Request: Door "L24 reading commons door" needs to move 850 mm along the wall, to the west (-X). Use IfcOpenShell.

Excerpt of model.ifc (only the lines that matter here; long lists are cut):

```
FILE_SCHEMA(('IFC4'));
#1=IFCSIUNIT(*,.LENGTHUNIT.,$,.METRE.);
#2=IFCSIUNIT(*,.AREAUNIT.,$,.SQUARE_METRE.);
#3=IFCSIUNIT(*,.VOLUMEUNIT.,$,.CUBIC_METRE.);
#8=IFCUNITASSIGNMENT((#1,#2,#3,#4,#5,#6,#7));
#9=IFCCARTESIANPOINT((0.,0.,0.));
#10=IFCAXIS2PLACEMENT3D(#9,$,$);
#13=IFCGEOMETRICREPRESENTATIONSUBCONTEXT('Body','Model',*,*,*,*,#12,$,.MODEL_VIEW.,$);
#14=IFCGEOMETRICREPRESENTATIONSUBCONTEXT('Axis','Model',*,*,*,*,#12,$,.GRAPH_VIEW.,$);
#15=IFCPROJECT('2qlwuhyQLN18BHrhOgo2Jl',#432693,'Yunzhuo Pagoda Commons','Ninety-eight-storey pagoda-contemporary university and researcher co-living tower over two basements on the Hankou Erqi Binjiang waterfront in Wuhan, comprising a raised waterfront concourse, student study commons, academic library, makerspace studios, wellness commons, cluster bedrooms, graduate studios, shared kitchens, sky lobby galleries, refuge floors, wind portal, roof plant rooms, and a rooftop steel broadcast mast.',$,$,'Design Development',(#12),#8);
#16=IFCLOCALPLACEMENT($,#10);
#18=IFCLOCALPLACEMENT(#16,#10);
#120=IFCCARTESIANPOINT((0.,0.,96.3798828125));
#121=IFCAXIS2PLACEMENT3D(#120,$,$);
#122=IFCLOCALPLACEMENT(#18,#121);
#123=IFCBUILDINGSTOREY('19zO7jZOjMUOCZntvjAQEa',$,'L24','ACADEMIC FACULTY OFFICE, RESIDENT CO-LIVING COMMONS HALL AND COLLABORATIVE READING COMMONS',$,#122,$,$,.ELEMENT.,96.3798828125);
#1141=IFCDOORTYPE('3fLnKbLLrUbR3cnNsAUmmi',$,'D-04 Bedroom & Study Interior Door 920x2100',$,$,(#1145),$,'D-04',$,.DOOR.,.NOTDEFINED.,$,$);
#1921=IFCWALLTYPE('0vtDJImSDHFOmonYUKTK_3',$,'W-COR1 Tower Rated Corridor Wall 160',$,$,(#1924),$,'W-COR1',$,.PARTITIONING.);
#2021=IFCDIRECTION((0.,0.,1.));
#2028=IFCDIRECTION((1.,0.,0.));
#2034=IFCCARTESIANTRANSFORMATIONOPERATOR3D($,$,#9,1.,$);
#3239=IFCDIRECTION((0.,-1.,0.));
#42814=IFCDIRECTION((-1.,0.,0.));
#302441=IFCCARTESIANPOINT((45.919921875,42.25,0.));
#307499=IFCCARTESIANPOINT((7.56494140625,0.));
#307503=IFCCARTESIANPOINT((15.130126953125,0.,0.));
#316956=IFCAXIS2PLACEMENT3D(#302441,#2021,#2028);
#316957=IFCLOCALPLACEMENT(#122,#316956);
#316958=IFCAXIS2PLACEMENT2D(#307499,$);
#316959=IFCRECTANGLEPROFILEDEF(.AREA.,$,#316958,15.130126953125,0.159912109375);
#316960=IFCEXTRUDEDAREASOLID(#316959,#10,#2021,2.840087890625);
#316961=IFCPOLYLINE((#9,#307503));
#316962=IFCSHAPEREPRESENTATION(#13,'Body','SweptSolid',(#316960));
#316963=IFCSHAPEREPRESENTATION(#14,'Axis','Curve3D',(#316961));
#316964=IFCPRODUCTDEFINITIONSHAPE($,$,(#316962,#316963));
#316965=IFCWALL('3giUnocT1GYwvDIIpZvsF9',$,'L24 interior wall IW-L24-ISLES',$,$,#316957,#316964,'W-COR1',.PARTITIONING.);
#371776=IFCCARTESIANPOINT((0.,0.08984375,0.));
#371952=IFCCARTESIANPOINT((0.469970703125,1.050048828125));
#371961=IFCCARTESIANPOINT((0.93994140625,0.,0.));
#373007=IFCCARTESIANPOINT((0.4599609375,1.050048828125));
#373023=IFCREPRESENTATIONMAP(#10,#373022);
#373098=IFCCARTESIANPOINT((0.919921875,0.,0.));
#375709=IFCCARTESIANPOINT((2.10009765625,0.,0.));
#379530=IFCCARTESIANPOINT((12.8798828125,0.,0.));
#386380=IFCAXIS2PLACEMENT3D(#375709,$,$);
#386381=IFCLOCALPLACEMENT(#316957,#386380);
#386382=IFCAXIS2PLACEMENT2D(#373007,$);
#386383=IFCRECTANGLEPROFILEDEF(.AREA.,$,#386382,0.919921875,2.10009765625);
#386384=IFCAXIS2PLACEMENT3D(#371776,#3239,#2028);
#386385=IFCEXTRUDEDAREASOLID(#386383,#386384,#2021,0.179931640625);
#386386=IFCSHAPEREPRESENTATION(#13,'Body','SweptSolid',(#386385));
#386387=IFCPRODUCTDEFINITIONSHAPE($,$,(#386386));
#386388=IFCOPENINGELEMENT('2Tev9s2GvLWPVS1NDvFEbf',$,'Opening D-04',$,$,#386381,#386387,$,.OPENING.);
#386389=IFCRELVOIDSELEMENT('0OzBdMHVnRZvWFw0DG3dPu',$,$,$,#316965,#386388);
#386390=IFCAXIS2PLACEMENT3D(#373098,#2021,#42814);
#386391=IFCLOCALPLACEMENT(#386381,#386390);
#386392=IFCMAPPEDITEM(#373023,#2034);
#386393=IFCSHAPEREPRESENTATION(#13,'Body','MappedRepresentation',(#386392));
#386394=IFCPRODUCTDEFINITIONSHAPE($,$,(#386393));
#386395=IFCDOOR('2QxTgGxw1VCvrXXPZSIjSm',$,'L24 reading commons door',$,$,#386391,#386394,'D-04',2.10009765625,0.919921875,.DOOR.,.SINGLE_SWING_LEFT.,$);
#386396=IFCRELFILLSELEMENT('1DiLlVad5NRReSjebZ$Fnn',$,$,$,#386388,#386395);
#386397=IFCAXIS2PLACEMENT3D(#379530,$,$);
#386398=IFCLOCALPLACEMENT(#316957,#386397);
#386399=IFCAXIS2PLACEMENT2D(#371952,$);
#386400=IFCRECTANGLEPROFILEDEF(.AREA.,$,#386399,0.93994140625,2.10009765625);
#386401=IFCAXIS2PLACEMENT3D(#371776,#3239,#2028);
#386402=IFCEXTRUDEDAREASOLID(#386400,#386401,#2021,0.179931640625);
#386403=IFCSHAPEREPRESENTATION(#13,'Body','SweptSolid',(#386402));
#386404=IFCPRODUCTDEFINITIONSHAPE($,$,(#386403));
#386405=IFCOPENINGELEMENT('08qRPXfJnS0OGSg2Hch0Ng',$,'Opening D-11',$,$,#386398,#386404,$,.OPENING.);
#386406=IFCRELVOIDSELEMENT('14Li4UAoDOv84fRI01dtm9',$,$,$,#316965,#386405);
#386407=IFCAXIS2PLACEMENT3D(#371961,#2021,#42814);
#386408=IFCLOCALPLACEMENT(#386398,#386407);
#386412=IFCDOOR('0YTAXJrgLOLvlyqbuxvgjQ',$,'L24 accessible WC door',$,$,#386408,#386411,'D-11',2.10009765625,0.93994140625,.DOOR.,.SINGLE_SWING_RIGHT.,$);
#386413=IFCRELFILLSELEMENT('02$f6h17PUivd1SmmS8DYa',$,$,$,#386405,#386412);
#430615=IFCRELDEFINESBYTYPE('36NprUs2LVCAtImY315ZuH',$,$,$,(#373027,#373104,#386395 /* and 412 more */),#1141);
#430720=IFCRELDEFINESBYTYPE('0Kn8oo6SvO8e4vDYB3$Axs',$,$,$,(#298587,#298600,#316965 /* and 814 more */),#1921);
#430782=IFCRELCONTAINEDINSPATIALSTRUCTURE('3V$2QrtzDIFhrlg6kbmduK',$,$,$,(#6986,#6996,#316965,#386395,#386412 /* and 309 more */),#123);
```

```python
import ifcopenshell
import ifcopenshell.api.geometry
import ifcopenshell.util.placement
import ifcopenshell.util.unit

model = ifcopenshell.open("model.ifc")
unit_scale = ifcopenshell.util.unit.calculate_unit_scale(model)

door = model.by_guid("2QxTgGxw1VCvrXXPZSIjSm")
opening = door.FillsVoids[0].RelatingOpeningElement
wall = opening.VoidsElements[0].RelatingBuildingElement

wall_matrix = ifcopenshell.util.placement.get_local_placement(wall.ObjectPlacement)
shift = wall_matrix[:3, 0] * -0.85 / unit_scale
before = ifcopenshell.util.placement.get_local_placement(door.ObjectPlacement)[:3, 3].copy()

# The door is placed relative to its opening, so it follows when the opening moves.
matrix = ifcopenshell.util.placement.get_local_placement(opening.ObjectPlacement)
matrix[:3, 3] += shift
ifcopenshell.api.geometry.edit_object_placement(
    model, product=opening, matrix=matrix, is_si=False, should_transform_children=True
)

after = ifcopenshell.util.placement.get_local_placement(door.ObjectPlacement)[:3, 3]
print("door moved by", (after - before).round(3) + 0.0)

model.write("model_rev.ifc")
```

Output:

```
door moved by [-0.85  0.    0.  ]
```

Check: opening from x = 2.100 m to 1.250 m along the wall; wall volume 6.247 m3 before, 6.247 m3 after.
